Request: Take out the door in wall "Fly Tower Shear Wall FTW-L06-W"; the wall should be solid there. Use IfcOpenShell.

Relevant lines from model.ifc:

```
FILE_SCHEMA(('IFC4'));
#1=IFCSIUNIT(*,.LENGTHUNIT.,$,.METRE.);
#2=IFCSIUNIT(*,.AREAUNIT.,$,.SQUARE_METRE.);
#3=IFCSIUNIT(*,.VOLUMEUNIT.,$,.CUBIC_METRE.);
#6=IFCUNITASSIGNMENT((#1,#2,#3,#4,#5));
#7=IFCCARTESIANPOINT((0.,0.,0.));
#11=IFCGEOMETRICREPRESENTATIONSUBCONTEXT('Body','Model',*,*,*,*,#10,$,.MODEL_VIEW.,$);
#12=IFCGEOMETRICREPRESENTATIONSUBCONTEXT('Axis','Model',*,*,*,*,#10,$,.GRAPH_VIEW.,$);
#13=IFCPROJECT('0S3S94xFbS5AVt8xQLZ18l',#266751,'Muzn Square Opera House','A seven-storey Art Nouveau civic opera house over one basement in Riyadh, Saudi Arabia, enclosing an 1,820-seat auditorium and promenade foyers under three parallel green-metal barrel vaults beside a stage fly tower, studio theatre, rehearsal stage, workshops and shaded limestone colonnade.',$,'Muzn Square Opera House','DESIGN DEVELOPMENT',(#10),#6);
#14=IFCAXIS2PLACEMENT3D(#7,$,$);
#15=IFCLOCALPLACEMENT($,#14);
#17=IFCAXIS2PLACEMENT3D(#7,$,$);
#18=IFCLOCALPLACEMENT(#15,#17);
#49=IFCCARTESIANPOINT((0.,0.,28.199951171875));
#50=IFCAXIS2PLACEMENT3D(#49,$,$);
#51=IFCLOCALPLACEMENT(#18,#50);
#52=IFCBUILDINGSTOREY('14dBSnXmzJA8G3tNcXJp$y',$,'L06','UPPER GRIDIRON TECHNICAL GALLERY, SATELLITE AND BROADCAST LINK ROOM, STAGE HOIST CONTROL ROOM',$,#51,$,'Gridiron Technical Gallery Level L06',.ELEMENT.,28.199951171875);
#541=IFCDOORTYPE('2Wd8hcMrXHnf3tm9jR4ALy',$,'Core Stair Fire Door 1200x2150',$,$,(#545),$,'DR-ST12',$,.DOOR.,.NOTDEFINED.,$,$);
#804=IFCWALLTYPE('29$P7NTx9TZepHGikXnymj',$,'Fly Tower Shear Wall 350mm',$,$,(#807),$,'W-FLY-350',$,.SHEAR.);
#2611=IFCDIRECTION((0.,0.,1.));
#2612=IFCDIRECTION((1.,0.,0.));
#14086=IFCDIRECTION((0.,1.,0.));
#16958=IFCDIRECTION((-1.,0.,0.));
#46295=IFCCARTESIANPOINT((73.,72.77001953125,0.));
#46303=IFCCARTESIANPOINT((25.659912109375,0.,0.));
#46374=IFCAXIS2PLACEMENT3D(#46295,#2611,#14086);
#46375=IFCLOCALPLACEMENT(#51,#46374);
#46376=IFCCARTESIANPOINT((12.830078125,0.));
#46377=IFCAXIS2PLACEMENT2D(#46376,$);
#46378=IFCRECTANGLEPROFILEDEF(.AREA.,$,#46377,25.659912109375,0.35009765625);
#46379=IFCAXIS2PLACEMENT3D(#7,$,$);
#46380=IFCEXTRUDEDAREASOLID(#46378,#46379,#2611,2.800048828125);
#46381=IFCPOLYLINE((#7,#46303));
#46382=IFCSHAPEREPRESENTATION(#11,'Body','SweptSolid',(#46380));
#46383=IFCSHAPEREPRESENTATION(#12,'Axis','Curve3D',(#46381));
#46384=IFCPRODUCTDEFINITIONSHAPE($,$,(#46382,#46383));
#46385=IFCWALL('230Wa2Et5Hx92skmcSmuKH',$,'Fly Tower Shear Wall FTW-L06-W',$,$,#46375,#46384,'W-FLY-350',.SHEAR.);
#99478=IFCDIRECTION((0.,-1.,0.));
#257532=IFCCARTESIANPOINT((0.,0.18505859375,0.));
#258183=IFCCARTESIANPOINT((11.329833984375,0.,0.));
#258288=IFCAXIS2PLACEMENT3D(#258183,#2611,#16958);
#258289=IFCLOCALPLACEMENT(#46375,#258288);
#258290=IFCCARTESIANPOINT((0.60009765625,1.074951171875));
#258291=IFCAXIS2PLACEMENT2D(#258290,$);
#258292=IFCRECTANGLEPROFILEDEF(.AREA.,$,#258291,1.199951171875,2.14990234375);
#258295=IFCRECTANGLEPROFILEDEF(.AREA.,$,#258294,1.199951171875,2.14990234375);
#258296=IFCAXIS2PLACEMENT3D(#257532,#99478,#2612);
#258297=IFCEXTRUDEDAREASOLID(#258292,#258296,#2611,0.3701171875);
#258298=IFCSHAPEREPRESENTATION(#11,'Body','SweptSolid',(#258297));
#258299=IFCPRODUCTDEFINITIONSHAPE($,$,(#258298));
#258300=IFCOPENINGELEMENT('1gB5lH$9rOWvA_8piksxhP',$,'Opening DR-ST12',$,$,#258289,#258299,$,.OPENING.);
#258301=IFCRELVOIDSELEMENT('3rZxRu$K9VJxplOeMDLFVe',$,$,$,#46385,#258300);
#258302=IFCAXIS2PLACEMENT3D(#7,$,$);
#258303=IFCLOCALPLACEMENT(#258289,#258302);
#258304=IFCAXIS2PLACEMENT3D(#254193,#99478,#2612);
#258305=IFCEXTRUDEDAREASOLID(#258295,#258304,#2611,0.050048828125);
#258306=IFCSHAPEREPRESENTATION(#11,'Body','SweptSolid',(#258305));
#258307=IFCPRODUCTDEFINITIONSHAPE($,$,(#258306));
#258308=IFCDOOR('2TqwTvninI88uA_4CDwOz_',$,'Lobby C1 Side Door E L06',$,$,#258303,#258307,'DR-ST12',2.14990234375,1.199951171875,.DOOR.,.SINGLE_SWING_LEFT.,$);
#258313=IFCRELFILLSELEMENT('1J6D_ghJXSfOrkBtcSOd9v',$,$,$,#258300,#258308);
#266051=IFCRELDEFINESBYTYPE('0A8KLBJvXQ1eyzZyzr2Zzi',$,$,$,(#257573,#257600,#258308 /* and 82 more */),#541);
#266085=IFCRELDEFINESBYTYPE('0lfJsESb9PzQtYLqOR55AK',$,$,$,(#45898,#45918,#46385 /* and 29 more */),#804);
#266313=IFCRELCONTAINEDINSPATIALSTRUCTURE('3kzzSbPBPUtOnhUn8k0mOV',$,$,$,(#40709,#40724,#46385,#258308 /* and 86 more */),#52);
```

```python
import ifcopenshell
import ifcopenshell.api.feature
import ifcopenshell.api.root
import ifcopenshell.geom
import ifcopenshell.util.shape

model = ifcopenshell.open("model.ifc")
settings = ifcopenshell.geom.settings()


def volume(element):
    """Net volume in cubic metres, openings subtracted."""
    shape = ifcopenshell.geom.create_shape(settings, element)
    return ifcopenshell.util.shape.get_volume(shape.geometry)


door = model.by_guid("2TqwTvninI88uA_4CDwOz_")
opening = door.FillsVoids[0].RelatingOpeningElement
wall = opening.VoidsElements[0].RelatingBuildingElement
before = volume(wall)

ifcopenshell.api.root.remove_product(model, product=door)
ifcopenshell.api.feature.remove_feature(model, feature=opening)

after = volume(wall)

print(f"wall volume {before:.3f} -> {after:.3f} m3")

model.write("model_updated.ifc")
```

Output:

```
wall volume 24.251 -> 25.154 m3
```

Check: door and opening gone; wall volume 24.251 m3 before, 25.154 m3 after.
